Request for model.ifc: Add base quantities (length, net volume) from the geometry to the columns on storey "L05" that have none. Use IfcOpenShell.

First a look at what the model holds.

```python
import ifcopenshell
import ifcopenshell.util.element
import ifcopenshell.util.unit

model = ifcopenshell.open("model.ifc")
print(model.schema)
for unit_type in ("LENGTHUNIT", "AREAUNIT", "VOLUMEUNIT"):
    print(unit_type, ifcopenshell.util.unit.calculate_unit_scale(model, unit_type))
storey = next(s for s in model.by_type("IfcBuildingStorey") if s.Name == "L05")
columns = [e for e in ifcopenshell.util.element.get_decomposition(storey) if e.is_a("IfcColumn")]
for e in sorted(columns, key=lambda e: e.id()):
    print(e.id(), e.is_a(), e.Name, list(ifcopenshell.util.element.get_psets(e, qtos_only=True)), sep=" | ")
```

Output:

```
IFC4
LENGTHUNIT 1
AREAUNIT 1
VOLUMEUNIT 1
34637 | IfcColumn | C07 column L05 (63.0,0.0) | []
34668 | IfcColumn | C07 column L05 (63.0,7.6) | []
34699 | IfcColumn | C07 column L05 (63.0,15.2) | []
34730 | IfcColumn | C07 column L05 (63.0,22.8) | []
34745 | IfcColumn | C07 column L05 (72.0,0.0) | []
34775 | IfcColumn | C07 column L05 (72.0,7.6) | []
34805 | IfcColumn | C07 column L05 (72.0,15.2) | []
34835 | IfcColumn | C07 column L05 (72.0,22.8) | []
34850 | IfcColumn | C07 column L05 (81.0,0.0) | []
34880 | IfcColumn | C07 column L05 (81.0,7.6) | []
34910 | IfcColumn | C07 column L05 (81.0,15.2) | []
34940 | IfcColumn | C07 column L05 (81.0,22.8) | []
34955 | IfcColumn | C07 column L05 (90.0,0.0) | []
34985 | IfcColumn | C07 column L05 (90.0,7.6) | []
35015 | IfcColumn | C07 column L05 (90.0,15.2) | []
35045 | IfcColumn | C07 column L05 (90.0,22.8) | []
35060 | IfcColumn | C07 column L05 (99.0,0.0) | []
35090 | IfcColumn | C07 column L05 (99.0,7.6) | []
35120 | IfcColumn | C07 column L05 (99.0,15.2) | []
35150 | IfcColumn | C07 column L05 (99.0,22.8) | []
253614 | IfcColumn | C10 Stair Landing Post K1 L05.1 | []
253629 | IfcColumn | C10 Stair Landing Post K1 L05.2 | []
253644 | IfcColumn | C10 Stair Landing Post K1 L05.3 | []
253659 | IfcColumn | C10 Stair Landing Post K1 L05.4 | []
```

```python
import ifcopenshell
import ifcopenshell.api.pset
import ifcopenshell.geom
import ifcopenshell.util.element
import ifcopenshell.util.shape
import ifcopenshell.util.unit

model = ifcopenshell.open("model.ifc")
unit_scale = ifcopenshell.util.unit.calculate_unit_scale(model)
volume_scale = ifcopenshell.util.unit.calculate_unit_scale(model, "VOLUMEUNIT")
settings = ifcopenshell.geom.settings()

storey = next(s for s in model.by_type("IfcBuildingStorey") if s.Name == "L05")
columns = [e for e in ifcopenshell.util.element.get_decomposition(storey) if e.is_a("IfcColumn")]

for e in sorted(columns, key=lambda e: e.id()):
    if ifcopenshell.util.element.get_psets(e, qtos_only=True, should_inherit=False):
        continue
    # Geometry comes back in metres, in the element's own axes.
    shape = ifcopenshell.geom.create_shape(settings, e)
    values = {
        "Length": ifcopenshell.util.shape.get_z(shape.geometry) / unit_scale,
        "NetVolume": ifcopenshell.util.shape.get_volume(shape.geometry) / volume_scale,
    }
    qto = ifcopenshell.api.pset.add_qto(model, product=e, name="Qto_ColumnBaseQuantities")
    ifcopenshell.api.pset.edit_qto(model, qto=qto, properties=values)
    print(e.id(), {k: round(v, 3) for k, v in values.items()})

model.write("model_edited.ifc")
```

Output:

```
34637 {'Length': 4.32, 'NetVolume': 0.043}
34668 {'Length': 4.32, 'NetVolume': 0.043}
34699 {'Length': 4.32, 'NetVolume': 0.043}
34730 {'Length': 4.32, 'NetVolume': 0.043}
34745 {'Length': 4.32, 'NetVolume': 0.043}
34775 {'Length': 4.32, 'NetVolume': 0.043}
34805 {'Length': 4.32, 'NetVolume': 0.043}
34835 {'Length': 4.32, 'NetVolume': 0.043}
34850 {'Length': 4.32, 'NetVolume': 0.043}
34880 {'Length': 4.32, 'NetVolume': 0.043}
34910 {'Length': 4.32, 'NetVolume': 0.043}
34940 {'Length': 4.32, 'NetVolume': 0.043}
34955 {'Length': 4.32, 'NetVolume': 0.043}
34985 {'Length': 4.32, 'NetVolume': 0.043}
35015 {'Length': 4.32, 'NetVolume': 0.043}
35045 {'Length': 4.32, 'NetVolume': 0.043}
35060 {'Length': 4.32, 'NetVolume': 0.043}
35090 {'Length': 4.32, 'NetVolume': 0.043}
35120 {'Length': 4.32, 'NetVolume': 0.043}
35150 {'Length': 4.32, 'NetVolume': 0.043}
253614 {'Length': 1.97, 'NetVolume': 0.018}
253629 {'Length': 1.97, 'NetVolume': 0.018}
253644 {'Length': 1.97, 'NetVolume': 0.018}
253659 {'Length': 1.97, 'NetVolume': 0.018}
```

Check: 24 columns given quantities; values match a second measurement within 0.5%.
